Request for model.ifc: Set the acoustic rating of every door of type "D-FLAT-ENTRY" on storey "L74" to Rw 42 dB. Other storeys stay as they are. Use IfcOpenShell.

First a look at what the model holds.

```python
import ifcopenshell
import ifcopenshell.util.element

model = ifcopenshell.open("model.ifc")
print(model.schema)
storey = next(s for s in model.by_type("IfcBuildingStorey") if s.Name == "L74")
doors = [e for e in ifcopenshell.util.element.get_decomposition(storey) if e.is_a("IfcDoor")]
seen = {}
for e in doors:
    element_type = ifcopenshell.util.element.get_type(e)
    key = (element_type.Name if element_type != e and element_type else None, ifcopenshell.util.element.get_pset(e, "Pset_DoorCommon", "AcousticRating"))
    seen[key] = seen.get(key, 0) + 1
for (name, value), count in sorted(seen.items(), key=str):
    print(count, "x", name, "|", value)
```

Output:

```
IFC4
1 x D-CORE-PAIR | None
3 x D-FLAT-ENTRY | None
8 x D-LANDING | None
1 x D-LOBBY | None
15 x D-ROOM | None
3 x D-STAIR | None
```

```python
import ifcopenshell
import ifcopenshell.api.pset
import ifcopenshell.util.element

model = ifcopenshell.open("model.ifc")

storey = next(s for s in model.by_type("IfcBuildingStorey") if s.Name == "L74")
doors = [e for e in ifcopenshell.util.element.get_decomposition(storey) if e.is_a("IfcDoor")]

count = 0
for e in doors:
    element_type = ifcopenshell.util.element.get_type(e)
    if element_type in (None, e) or element_type.Name != "D-FLAT-ENTRY":
        continue
    found = ifcopenshell.util.element.get_pset(e, "Pset_DoorCommon", should_inherit=False)
    if found:
        pset = model.by_id(found["id"])
        if len(ifcopenshell.util.element.get_elements_by_pset(pset)) > 1:
            pset = ifcopenshell.api.pset.unshare_pset(model, products=[e], pset=pset)[0]
    else:
        pset = ifcopenshell.api.pset.add_pset(model, product=e, name="Pset_DoorCommon")
    ifcopenshell.api.pset.edit_pset(model, pset=pset, properties={"AcousticRating": "Rw 42 dB"})
    count += 1

print(count, "doors updated")

model.write("model_rev.ifc")
```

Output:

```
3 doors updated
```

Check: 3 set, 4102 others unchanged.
